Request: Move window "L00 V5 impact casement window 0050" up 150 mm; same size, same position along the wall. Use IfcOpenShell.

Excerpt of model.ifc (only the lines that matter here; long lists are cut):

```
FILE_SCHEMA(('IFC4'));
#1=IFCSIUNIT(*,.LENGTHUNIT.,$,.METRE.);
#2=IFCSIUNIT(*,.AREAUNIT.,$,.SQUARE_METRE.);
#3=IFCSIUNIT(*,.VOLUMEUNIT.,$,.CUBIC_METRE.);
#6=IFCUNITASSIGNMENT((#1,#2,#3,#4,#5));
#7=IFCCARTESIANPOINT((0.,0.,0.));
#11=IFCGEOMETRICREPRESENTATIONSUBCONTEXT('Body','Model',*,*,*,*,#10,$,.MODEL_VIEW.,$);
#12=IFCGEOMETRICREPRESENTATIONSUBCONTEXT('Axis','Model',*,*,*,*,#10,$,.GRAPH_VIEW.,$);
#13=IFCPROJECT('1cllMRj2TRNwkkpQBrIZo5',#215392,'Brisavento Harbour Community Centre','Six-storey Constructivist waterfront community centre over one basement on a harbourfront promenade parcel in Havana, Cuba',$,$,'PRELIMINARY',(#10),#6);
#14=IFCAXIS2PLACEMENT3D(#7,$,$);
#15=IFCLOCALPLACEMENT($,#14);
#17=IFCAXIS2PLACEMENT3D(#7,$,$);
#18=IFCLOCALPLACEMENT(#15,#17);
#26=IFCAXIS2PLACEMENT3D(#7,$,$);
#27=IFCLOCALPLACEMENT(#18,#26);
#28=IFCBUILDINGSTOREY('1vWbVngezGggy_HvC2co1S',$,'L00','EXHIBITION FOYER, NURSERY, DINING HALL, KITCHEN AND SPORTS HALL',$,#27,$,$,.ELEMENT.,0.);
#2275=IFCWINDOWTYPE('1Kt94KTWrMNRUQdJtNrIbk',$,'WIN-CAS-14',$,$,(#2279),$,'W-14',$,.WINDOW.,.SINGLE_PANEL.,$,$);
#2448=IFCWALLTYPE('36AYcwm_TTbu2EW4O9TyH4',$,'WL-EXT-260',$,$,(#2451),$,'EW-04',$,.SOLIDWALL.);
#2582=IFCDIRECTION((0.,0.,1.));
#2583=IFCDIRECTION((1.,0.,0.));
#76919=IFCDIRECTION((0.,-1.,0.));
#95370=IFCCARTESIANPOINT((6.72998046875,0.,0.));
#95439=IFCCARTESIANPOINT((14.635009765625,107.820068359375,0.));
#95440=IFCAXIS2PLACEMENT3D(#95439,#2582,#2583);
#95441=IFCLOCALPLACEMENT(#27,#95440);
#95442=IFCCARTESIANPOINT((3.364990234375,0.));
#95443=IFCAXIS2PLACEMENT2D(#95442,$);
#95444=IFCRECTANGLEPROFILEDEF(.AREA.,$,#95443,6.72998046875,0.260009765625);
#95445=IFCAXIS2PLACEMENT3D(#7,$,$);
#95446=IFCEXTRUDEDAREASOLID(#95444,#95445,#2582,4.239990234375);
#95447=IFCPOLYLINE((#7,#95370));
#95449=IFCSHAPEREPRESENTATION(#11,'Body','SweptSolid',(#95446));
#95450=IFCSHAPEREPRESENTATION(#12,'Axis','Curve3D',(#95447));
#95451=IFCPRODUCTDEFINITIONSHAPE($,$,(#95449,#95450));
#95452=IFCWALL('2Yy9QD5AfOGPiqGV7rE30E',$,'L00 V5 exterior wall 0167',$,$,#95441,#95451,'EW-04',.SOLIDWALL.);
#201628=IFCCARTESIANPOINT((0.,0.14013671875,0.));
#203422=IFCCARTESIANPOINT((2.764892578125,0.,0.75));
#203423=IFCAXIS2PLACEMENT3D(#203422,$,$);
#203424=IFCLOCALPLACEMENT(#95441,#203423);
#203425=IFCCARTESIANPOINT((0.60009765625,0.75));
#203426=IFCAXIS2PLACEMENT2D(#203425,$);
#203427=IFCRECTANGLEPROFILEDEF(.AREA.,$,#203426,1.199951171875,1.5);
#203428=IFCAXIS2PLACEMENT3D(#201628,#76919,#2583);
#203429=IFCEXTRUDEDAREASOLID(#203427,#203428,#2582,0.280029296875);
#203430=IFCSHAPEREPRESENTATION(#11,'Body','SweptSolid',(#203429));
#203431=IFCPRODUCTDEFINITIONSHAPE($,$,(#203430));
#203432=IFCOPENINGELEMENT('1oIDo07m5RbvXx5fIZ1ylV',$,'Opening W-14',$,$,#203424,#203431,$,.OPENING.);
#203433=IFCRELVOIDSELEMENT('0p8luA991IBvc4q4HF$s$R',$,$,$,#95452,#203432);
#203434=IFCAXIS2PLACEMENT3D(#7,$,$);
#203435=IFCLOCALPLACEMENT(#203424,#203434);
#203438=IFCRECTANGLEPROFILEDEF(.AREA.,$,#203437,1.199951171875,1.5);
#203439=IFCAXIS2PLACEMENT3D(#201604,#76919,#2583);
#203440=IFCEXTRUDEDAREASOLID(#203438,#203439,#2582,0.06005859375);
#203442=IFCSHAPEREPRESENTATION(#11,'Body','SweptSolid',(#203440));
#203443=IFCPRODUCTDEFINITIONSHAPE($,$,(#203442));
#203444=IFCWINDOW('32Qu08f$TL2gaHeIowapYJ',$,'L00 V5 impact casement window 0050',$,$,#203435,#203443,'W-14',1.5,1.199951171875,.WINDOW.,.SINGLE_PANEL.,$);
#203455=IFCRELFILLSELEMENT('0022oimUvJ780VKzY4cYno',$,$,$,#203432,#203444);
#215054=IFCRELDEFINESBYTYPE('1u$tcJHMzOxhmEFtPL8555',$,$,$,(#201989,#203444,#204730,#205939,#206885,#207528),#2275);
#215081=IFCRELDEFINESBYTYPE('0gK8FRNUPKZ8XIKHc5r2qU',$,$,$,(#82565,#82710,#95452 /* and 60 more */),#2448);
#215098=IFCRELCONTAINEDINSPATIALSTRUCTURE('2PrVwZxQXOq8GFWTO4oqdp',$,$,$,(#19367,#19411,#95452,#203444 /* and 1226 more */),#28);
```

```python
import numpy as np
import ifcopenshell
import ifcopenshell.api.geometry
import ifcopenshell.util.placement
import ifcopenshell.util.unit

model = ifcopenshell.open("model.ifc")
unit_scale = ifcopenshell.util.unit.calculate_unit_scale(model)

window = model.by_guid("32Qu08f$TL2gaHeIowapYJ")
opening = window.FillsVoids[0].RelatingOpeningElement
dz = 0.15

shift = np.array([0.0, 0.0, dz])
# The window is placed relative to its opening, so it follows when the opening moves.
matrix = ifcopenshell.util.placement.get_local_placement(opening.ObjectPlacement)
matrix[:3, 3] += shift
ifcopenshell.api.geometry.edit_object_placement(
    model, product=opening, matrix=matrix, is_si=False, should_transform_children=True
)

print(f"moved by {dz * unit_scale:+.3f} m")

model.write("model_v2.ifc")
```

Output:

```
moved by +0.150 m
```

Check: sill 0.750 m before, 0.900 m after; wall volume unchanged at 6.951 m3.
